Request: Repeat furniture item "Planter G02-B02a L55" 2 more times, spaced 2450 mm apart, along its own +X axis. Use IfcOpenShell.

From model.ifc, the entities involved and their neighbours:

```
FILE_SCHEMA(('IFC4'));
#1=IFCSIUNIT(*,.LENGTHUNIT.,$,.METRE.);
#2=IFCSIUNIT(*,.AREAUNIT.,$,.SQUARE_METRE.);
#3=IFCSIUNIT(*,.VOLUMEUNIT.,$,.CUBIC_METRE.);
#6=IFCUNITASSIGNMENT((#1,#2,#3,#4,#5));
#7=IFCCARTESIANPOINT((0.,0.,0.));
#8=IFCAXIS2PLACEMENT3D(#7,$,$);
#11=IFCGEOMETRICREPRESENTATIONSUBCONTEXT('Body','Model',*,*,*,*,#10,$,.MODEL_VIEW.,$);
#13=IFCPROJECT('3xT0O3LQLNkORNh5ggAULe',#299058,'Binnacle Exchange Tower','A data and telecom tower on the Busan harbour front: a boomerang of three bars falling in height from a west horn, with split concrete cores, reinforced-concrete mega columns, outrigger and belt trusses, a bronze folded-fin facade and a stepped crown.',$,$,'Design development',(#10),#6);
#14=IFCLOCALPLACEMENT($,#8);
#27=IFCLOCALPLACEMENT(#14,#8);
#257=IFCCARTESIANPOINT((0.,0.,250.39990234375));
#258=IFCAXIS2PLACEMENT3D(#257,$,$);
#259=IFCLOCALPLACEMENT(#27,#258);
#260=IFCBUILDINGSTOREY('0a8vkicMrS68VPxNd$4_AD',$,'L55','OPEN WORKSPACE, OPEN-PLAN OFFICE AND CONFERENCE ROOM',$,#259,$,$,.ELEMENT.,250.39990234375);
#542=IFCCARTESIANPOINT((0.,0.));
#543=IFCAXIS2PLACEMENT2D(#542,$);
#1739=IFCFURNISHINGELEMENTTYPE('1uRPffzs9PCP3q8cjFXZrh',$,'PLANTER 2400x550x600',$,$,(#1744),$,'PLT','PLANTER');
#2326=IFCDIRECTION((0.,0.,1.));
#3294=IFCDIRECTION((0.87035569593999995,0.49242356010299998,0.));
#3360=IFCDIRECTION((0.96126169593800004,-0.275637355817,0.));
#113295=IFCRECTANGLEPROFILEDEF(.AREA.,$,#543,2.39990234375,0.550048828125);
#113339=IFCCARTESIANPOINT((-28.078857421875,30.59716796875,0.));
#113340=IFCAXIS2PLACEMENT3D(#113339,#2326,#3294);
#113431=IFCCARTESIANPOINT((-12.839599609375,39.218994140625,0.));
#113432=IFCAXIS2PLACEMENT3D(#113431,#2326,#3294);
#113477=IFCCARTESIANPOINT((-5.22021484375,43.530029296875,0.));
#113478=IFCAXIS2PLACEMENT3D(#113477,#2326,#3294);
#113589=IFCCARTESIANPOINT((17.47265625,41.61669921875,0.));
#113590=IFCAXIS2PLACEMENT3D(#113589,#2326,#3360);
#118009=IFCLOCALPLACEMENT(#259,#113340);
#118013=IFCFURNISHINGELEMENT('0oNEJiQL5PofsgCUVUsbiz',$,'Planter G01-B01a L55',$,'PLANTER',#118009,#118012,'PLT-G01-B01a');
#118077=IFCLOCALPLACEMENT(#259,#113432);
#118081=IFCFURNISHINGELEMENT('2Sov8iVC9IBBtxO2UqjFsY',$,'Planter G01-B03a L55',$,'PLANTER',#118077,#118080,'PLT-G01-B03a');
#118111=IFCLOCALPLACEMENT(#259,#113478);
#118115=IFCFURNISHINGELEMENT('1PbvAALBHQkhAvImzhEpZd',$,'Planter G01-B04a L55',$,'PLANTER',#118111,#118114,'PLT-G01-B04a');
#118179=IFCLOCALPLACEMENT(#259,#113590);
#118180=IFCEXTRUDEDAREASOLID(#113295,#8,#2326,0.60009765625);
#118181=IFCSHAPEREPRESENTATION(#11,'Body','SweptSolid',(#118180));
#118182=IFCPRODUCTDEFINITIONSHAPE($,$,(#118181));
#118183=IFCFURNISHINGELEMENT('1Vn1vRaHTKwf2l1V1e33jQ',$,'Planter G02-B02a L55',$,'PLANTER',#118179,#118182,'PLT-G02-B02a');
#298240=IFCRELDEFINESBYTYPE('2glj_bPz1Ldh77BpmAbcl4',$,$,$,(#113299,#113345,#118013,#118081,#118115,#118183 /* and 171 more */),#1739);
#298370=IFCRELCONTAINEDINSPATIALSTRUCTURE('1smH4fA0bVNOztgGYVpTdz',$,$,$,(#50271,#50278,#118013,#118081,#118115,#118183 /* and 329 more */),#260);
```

```python
import ifcopenshell
import ifcopenshell.api.geometry
import ifcopenshell.api.root
import ifcopenshell.util.element
import ifcopenshell.util.placement
import ifcopenshell.util.unit

model = ifcopenshell.open("model.ifc")
unit_scale = ifcopenshell.util.unit.calculate_unit_scale(model)

source = model.by_id(118183)
base = ifcopenshell.util.placement.get_local_placement(source.ObjectPlacement)
step = base[:3, 0] * 2.45 / unit_scale

for i in range(1, 3):
    copy = ifcopenshell.api.root.copy_class(model, product=source)
    copy.Representation = ifcopenshell.util.element.copy_deep(
        model, source.Representation, exclude=["IfcGeometricRepresentationContext", "IfcRepresentationMap"]
    )
    copy.Tag = None
    matrix = base.copy()
    matrix[:3, 3] += i * step
    print("added at", matrix[:3, 3].round(3) + 0.0)
    ifcopenshell.api.geometry.edit_object_placement(model, product=copy, matrix=matrix, is_si=False)

model.write("model_updated.ifc")
```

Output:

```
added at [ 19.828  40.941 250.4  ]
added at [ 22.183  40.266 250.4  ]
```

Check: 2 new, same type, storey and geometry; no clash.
